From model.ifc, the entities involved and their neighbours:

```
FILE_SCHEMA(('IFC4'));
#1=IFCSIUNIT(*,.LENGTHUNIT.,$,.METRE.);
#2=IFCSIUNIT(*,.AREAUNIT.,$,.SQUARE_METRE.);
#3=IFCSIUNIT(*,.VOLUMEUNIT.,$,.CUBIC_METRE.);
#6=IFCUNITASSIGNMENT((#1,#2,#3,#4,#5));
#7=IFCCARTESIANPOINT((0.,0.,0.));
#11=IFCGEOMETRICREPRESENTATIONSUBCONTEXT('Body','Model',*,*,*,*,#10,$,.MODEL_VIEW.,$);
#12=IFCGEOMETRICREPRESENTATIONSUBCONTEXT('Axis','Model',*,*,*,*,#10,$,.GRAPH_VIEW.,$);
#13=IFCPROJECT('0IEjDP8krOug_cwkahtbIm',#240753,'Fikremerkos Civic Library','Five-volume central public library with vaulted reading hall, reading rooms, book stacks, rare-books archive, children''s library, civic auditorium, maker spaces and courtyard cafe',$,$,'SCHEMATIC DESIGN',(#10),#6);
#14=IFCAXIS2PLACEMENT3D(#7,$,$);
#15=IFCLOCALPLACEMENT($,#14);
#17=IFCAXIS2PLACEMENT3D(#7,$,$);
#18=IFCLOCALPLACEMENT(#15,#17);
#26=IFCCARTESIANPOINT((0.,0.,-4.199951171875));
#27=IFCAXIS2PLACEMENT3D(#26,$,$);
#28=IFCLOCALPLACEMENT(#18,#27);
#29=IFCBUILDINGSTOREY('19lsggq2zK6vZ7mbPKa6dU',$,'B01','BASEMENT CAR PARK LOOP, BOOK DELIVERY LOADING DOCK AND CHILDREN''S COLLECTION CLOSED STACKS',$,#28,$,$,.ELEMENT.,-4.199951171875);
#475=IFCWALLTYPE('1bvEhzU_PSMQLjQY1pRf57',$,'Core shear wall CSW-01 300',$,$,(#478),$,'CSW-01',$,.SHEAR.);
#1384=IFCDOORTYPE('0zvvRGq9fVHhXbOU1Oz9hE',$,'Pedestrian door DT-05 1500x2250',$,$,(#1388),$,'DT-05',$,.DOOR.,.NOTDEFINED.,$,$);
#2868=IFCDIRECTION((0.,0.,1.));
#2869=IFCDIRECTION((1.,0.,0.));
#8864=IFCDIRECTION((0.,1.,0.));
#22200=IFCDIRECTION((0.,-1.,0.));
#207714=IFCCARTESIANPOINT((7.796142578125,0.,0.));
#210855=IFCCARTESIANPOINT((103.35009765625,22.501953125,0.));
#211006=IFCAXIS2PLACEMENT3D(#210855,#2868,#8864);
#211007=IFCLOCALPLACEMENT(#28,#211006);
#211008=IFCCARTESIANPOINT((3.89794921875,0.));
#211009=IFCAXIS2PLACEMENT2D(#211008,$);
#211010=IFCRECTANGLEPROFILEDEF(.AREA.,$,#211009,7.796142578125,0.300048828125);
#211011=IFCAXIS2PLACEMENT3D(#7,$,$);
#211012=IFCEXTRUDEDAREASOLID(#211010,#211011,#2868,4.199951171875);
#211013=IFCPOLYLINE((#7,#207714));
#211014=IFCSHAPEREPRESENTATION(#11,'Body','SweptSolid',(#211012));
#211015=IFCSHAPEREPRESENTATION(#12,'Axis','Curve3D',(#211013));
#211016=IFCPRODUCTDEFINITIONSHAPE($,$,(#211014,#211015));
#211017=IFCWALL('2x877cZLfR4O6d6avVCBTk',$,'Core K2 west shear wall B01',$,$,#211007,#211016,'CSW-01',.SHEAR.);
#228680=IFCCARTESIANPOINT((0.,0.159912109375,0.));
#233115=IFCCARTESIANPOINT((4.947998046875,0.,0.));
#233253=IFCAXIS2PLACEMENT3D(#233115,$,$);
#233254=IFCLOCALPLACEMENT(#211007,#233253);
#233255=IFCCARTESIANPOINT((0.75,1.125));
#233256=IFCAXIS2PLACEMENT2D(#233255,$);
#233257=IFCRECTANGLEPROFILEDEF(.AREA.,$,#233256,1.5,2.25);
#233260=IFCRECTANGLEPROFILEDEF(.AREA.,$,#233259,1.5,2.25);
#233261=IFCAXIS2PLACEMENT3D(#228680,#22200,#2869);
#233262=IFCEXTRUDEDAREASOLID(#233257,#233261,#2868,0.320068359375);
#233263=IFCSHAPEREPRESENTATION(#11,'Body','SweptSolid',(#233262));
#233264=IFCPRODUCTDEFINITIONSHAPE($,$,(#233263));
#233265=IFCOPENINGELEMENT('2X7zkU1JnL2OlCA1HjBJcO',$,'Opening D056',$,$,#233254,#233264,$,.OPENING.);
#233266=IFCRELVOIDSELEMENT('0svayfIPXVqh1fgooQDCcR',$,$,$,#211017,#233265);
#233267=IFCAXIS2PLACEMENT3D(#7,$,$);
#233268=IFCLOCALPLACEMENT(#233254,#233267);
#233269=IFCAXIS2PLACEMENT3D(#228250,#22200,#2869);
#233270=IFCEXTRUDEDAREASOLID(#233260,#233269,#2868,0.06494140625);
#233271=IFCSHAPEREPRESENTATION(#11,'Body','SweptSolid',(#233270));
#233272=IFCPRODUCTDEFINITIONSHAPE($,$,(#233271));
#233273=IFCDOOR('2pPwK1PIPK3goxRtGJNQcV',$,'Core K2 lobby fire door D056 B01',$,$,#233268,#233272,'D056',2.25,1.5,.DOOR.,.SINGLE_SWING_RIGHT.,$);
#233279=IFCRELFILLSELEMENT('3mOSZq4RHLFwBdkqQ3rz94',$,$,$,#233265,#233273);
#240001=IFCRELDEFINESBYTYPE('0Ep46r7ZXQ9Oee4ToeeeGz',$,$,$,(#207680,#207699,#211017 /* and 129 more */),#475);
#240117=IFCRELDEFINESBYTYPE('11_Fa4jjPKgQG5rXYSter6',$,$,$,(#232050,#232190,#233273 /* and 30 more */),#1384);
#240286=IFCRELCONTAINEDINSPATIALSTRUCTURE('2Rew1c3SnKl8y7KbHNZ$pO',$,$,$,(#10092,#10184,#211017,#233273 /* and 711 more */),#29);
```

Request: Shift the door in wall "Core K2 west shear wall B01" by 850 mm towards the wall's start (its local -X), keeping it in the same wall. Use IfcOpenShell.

```python
import ifcopenshell
import ifcopenshell.api.geometry
import ifcopenshell.util.placement

model = ifcopenshell.open("model.ifc")

door = model.by_guid("2pPwK1PIPK3goxRtGJNQcV")
opening = door.FillsVoids[0].RelatingOpeningElement
wall = opening.VoidsElements[0].RelatingBuildingElement

wall_matrix = ifcopenshell.util.placement.get_local_placement(wall.ObjectPlacement)
shift = wall_matrix[:3, 0] * -0.85
before = ifcopenshell.util.placement.get_local_placement(door.ObjectPlacement)[:3, 3].copy()

# The door is placed relative to its opening, so it follows when the opening moves.
matrix = ifcopenshell.util.placement.get_local_placement(opening.ObjectPlacement)
matrix[:3, 3] += shift
ifcopenshell.api.geometry.edit_object_placement(
    model, product=opening, matrix=matrix, is_si=False, should_transform_children=True
)

after = ifcopenshell.util.placement.get_local_placement(door.ObjectPlacement)[:3, 3]
print("door moved by", (after - before).round(3) + 0.0)

model.write("model_v2.ifc")
```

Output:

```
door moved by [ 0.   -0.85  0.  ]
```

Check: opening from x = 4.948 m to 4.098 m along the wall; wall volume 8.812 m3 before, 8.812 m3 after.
